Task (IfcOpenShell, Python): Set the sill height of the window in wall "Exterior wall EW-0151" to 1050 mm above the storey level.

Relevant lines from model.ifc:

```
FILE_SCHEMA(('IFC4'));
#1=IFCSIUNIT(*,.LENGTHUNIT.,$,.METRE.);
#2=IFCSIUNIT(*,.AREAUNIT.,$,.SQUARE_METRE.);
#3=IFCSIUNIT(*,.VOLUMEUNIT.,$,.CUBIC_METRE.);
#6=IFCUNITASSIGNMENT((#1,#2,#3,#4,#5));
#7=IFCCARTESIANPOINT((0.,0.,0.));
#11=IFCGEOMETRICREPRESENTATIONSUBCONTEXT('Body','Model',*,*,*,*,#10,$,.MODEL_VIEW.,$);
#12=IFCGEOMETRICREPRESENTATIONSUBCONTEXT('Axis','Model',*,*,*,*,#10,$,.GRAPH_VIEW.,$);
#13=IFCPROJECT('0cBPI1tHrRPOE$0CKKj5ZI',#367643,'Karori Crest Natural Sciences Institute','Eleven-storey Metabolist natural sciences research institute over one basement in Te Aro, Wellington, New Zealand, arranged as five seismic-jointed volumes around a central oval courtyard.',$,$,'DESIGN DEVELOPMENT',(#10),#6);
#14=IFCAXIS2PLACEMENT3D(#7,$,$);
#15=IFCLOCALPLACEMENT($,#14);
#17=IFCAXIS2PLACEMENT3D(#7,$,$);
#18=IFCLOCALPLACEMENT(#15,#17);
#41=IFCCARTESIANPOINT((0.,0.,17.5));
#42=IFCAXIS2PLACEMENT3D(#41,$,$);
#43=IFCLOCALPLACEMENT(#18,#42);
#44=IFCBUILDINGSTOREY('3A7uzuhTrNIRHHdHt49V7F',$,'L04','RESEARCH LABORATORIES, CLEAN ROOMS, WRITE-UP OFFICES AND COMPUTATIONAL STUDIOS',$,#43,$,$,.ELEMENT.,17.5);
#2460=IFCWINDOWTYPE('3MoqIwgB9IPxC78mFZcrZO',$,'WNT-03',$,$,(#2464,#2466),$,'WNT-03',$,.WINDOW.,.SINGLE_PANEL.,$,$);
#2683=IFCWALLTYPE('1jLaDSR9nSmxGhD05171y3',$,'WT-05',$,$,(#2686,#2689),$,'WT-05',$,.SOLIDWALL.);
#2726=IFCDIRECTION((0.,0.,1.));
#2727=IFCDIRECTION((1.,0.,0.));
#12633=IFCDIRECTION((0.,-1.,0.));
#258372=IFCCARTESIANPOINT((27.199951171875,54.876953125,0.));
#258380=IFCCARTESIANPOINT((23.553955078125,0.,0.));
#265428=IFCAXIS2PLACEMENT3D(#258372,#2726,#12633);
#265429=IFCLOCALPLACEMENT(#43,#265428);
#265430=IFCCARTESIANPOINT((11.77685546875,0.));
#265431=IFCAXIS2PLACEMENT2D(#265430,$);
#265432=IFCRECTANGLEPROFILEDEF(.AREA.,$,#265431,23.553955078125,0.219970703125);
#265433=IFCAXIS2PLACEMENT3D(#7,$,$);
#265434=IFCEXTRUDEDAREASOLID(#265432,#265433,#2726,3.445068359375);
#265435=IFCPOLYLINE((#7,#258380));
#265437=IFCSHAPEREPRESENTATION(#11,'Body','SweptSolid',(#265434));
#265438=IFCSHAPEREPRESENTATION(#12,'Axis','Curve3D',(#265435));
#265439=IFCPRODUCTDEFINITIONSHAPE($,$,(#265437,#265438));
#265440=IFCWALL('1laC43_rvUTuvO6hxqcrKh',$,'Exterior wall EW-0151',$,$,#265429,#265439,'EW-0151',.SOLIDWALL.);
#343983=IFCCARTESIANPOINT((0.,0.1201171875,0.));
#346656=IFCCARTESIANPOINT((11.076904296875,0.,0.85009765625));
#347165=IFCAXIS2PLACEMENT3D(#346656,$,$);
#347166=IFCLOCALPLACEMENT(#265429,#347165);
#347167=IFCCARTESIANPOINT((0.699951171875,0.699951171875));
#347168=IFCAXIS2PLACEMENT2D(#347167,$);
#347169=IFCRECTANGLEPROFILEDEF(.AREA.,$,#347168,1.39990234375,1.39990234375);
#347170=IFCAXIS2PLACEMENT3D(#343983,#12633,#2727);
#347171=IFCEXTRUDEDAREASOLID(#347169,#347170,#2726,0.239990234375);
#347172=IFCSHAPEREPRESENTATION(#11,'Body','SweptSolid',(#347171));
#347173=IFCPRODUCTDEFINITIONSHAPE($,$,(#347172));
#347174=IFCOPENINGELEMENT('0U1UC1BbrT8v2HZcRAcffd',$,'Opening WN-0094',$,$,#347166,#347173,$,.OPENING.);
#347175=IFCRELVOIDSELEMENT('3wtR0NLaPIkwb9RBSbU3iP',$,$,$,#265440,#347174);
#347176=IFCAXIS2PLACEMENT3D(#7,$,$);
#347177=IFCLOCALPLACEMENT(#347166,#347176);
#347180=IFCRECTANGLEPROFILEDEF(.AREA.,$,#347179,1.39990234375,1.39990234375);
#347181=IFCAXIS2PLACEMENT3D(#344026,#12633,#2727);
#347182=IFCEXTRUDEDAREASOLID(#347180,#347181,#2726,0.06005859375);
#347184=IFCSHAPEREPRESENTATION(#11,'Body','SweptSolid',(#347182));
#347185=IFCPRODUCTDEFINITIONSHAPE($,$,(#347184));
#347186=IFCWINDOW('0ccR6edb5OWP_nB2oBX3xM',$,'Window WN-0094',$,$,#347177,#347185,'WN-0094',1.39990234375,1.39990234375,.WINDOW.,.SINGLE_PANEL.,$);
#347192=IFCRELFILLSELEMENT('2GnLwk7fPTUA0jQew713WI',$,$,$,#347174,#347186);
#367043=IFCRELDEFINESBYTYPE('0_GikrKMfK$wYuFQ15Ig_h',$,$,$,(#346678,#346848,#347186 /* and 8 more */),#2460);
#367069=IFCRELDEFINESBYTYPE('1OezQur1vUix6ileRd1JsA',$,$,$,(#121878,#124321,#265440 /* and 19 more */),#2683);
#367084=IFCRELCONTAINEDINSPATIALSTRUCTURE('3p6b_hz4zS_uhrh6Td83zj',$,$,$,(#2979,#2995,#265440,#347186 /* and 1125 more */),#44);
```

```python
import numpy as np
import ifcopenshell
import ifcopenshell.api.geometry
import ifcopenshell.geom
import ifcopenshell.util.element
import ifcopenshell.util.placement
import ifcopenshell.util.shape
import ifcopenshell.util.unit

model = ifcopenshell.open("model.ifc")
unit_scale = ifcopenshell.util.unit.calculate_unit_scale(model)

window = model.by_id(347186)
opening = window.FillsVoids[0].RelatingOpeningElement
storey = ifcopenshell.util.element.get_container(window, ifc_class="IfcBuildingStorey")
level = ifcopenshell.util.placement.get_local_placement(storey.ObjectPlacement)[2, 3]

# The opening's origin need not be at the sill, so measure its lowest point.
shape = ifcopenshell.geom.create_shape(ifcopenshell.geom.settings(), opening)
bottom = ifcopenshell.util.shape.get_shape_bottom_elevation(shape, shape.geometry) / unit_scale
dz = level + 1.05 / unit_scale - bottom

shift = np.array([0.0, 0.0, dz])
# The window is placed relative to its opening, so it follows when the opening moves.
matrix = ifcopenshell.util.placement.get_local_placement(opening.ObjectPlacement)
matrix[:3, 3] += shift
ifcopenshell.api.geometry.edit_object_placement(
    model, product=opening, matrix=matrix, is_si=False, should_transform_children=True
)

print(f"moved by {dz * unit_scale:+.3f} m")

model.write("model_v2.ifc")
```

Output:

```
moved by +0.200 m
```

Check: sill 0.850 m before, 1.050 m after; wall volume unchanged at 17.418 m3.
